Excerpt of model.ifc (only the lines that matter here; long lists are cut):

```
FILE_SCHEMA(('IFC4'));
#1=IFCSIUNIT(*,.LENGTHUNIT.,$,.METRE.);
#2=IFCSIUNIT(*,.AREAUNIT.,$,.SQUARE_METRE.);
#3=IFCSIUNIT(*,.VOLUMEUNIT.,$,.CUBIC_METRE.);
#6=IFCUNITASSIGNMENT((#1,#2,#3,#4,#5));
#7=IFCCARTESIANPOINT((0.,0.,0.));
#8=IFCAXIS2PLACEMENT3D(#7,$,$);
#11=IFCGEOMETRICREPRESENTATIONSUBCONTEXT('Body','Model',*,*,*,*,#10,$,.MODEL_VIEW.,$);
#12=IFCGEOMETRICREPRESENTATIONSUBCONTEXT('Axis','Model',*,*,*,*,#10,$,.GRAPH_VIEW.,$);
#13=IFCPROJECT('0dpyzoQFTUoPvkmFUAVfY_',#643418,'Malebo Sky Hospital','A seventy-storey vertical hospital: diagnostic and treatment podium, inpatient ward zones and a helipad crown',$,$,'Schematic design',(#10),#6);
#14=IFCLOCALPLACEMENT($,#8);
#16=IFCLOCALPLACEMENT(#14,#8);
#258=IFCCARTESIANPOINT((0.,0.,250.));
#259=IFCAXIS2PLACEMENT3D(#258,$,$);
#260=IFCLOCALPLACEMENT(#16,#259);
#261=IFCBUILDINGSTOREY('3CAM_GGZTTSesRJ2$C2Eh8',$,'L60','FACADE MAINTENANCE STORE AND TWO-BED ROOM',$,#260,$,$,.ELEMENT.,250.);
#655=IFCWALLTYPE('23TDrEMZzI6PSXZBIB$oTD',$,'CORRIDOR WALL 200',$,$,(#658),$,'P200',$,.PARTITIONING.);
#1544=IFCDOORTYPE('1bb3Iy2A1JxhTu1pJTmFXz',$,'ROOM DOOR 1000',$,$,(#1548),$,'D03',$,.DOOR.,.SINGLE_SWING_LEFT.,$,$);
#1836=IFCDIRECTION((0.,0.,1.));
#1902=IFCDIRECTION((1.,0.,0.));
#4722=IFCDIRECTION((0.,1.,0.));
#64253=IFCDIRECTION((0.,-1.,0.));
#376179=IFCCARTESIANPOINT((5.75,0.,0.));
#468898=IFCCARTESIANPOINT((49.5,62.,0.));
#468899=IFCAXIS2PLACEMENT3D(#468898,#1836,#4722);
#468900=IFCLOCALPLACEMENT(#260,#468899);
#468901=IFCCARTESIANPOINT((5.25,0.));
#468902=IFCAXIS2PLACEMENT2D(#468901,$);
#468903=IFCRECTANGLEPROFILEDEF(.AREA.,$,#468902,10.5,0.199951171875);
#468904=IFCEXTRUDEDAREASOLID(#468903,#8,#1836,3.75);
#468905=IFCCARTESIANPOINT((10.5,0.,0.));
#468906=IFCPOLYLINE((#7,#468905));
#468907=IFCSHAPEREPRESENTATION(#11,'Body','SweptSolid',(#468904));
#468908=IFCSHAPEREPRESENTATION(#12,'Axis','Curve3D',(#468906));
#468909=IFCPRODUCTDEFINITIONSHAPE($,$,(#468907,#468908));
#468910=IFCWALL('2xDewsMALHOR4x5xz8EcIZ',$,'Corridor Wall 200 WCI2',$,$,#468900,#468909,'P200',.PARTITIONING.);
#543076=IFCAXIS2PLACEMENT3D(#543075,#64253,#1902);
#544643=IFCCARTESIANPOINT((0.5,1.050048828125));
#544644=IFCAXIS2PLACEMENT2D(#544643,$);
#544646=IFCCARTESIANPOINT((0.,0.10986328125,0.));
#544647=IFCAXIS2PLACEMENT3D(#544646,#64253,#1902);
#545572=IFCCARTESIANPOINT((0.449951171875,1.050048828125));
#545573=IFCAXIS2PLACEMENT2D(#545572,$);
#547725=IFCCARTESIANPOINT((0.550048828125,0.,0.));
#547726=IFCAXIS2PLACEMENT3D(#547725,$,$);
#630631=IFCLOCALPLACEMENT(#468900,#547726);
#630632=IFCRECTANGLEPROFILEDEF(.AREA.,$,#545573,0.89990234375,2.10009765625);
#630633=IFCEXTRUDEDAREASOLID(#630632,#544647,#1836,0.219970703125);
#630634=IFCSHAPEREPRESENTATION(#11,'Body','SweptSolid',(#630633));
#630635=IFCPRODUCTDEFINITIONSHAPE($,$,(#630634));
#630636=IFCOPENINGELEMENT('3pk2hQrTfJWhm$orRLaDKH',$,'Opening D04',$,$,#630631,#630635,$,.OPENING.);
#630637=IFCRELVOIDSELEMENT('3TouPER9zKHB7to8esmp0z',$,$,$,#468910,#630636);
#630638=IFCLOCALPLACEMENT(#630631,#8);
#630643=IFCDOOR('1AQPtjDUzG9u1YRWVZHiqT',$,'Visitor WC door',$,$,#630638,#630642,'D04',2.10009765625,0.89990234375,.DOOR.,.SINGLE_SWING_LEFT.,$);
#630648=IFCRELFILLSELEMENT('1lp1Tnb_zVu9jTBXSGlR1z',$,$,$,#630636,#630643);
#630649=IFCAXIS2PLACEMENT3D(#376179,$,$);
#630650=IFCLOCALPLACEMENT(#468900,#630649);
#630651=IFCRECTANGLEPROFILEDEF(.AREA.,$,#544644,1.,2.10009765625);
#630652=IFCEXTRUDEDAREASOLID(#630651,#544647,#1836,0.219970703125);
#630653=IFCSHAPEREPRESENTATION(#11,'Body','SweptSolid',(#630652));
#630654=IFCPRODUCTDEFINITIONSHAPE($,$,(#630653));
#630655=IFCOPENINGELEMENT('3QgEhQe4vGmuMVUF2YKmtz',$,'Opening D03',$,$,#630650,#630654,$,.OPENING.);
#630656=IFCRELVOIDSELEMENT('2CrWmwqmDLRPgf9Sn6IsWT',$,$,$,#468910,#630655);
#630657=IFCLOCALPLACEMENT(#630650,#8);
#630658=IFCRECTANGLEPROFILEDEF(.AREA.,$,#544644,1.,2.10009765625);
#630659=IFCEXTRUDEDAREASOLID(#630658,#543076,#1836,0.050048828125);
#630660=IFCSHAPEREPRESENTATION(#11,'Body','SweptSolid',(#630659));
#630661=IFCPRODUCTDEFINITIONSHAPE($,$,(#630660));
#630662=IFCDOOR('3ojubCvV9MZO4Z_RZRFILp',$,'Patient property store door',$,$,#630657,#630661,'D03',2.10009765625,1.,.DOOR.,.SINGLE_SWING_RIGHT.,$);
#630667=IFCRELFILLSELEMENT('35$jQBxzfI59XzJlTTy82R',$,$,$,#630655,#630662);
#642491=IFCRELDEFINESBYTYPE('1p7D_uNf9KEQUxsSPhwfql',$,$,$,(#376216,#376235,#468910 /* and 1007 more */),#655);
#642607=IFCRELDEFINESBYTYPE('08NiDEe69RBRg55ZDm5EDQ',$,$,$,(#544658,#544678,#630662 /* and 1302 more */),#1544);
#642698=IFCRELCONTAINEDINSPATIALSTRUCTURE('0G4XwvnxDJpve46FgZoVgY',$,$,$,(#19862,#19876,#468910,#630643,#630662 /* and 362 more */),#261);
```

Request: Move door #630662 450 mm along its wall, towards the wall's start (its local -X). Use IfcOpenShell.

```python
import ifcopenshell
import ifcopenshell.api.geometry
import ifcopenshell.util.placement

model = ifcopenshell.open("model.ifc")

door = model.by_guid("3ojubCvV9MZO4Z_RZRFILp")
opening = door.FillsVoids[0].RelatingOpeningElement
wall = opening.VoidsElements[0].RelatingBuildingElement

wall_matrix = ifcopenshell.util.placement.get_local_placement(wall.ObjectPlacement)
shift = wall_matrix[:3, 0] * -0.45
before = ifcopenshell.util.placement.get_local_placement(door.ObjectPlacement)[:3, 3].copy()

# The door is placed relative to its opening, so it follows when the opening moves.
matrix = ifcopenshell.util.placement.get_local_placement(opening.ObjectPlacement)
matrix[:3, 3] += shift
ifcopenshell.api.geometry.edit_object_placement(
    model, product=opening, matrix=matrix, is_si=False, should_transform_children=True
)

after = ifcopenshell.util.placement.get_local_placement(door.ObjectPlacement)[:3, 3]
print("door moved by", (after - before).round(3) + 0.0)

model.write("model_edited.ifc")
```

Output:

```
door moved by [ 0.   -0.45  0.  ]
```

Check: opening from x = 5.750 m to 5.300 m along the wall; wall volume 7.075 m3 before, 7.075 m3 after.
